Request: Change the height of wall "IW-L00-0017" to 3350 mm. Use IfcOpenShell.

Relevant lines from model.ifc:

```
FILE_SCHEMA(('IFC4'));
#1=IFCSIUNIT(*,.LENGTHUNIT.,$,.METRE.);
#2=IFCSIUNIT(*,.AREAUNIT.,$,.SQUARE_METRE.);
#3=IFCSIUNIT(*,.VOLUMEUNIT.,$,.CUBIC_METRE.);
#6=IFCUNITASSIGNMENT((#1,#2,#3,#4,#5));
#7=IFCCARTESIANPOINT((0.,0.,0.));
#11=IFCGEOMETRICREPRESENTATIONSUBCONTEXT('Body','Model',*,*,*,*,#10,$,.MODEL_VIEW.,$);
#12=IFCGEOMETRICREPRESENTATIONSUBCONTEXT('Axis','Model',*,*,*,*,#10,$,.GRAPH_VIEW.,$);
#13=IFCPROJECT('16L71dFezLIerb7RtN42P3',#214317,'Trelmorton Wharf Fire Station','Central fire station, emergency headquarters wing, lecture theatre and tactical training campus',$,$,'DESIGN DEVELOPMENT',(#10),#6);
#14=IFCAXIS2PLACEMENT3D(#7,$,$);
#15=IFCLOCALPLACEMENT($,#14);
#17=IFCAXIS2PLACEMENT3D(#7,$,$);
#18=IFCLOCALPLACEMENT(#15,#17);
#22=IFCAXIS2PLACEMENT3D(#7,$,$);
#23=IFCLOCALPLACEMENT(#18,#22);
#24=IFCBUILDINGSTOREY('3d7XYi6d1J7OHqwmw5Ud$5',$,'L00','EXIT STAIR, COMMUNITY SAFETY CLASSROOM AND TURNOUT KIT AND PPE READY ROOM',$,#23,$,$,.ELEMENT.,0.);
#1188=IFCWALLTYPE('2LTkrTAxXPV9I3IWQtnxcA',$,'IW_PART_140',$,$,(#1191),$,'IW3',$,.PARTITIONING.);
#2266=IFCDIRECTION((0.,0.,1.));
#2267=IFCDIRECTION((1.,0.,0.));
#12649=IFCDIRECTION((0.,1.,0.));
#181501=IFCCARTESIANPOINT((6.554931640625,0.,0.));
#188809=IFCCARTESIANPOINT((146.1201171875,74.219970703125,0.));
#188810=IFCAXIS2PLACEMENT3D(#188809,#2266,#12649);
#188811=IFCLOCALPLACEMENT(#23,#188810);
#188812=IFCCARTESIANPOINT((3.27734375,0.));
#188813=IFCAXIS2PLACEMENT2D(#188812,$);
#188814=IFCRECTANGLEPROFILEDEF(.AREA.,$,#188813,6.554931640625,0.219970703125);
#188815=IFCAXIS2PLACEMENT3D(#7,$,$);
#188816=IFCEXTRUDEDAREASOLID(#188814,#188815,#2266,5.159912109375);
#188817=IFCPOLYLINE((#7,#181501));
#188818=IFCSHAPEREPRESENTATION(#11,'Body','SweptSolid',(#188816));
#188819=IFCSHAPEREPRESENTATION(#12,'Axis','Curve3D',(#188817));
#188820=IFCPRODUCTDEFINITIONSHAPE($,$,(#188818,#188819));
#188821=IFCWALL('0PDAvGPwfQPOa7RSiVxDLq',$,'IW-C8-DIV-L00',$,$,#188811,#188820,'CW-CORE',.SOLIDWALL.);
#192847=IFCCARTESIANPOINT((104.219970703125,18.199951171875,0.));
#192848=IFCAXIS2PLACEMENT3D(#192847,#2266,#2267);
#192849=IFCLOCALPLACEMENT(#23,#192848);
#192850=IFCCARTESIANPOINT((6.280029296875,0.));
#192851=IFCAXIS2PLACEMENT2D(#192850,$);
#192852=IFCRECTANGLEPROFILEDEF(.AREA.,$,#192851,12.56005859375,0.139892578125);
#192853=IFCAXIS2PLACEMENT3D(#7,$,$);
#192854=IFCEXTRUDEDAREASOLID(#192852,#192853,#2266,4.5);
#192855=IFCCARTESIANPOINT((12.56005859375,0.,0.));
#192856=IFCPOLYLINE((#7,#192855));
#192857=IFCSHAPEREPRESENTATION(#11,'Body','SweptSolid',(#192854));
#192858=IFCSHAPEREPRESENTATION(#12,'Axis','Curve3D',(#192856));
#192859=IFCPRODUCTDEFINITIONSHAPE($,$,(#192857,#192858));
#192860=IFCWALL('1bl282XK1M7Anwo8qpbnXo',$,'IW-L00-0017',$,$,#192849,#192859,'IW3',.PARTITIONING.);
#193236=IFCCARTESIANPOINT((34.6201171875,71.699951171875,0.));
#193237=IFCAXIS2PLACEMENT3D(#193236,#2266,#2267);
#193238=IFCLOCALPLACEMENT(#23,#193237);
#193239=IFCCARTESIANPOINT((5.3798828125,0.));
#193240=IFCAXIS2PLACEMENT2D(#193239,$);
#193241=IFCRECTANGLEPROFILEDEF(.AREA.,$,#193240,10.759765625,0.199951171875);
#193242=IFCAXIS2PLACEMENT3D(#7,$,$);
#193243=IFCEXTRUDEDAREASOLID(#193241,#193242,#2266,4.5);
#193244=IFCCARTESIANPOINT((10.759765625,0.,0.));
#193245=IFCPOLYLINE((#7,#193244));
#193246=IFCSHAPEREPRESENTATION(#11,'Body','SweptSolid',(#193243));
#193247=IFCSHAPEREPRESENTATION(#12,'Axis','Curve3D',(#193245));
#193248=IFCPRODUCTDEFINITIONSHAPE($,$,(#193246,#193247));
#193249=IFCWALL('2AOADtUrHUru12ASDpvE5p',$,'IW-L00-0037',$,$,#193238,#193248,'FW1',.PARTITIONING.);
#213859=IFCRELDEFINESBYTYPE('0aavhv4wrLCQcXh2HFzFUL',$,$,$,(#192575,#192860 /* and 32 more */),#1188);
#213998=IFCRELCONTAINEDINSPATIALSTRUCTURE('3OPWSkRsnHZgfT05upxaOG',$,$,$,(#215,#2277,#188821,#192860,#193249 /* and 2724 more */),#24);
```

```python
import ifcopenshell
import ifcopenshell.geom
import ifcopenshell.util.representation
import ifcopenshell.util.shape
import ifcopenshell.util.unit

model = ifcopenshell.open("model.ifc")
unit_scale = ifcopenshell.util.unit.calculate_unit_scale(model)
settings = ifcopenshell.geom.settings()


def volume(element):
    """Net volume in cubic metres, openings subtracted."""
    shape = ifcopenshell.geom.create_shape(settings, element)
    return ifcopenshell.util.shape.get_volume(shape.geometry)


wall = model.by_guid("1bl282XK1M7Anwo8qpbnXo")
before = volume(wall)

body = ifcopenshell.util.representation.get_representation(wall, "Model", "Body")
solid = body.Items[0]
old_height = solid.Depth
solid.Depth = 3.35 / unit_scale
after = volume(wall)

print(f"height {old_height:g} -> {solid.Depth:g}, volume {before:.3f} -> {after:.3f} m3")

model.write("model_rev.ifc")
```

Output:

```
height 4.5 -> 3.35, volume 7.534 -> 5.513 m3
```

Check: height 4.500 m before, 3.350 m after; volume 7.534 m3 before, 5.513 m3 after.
